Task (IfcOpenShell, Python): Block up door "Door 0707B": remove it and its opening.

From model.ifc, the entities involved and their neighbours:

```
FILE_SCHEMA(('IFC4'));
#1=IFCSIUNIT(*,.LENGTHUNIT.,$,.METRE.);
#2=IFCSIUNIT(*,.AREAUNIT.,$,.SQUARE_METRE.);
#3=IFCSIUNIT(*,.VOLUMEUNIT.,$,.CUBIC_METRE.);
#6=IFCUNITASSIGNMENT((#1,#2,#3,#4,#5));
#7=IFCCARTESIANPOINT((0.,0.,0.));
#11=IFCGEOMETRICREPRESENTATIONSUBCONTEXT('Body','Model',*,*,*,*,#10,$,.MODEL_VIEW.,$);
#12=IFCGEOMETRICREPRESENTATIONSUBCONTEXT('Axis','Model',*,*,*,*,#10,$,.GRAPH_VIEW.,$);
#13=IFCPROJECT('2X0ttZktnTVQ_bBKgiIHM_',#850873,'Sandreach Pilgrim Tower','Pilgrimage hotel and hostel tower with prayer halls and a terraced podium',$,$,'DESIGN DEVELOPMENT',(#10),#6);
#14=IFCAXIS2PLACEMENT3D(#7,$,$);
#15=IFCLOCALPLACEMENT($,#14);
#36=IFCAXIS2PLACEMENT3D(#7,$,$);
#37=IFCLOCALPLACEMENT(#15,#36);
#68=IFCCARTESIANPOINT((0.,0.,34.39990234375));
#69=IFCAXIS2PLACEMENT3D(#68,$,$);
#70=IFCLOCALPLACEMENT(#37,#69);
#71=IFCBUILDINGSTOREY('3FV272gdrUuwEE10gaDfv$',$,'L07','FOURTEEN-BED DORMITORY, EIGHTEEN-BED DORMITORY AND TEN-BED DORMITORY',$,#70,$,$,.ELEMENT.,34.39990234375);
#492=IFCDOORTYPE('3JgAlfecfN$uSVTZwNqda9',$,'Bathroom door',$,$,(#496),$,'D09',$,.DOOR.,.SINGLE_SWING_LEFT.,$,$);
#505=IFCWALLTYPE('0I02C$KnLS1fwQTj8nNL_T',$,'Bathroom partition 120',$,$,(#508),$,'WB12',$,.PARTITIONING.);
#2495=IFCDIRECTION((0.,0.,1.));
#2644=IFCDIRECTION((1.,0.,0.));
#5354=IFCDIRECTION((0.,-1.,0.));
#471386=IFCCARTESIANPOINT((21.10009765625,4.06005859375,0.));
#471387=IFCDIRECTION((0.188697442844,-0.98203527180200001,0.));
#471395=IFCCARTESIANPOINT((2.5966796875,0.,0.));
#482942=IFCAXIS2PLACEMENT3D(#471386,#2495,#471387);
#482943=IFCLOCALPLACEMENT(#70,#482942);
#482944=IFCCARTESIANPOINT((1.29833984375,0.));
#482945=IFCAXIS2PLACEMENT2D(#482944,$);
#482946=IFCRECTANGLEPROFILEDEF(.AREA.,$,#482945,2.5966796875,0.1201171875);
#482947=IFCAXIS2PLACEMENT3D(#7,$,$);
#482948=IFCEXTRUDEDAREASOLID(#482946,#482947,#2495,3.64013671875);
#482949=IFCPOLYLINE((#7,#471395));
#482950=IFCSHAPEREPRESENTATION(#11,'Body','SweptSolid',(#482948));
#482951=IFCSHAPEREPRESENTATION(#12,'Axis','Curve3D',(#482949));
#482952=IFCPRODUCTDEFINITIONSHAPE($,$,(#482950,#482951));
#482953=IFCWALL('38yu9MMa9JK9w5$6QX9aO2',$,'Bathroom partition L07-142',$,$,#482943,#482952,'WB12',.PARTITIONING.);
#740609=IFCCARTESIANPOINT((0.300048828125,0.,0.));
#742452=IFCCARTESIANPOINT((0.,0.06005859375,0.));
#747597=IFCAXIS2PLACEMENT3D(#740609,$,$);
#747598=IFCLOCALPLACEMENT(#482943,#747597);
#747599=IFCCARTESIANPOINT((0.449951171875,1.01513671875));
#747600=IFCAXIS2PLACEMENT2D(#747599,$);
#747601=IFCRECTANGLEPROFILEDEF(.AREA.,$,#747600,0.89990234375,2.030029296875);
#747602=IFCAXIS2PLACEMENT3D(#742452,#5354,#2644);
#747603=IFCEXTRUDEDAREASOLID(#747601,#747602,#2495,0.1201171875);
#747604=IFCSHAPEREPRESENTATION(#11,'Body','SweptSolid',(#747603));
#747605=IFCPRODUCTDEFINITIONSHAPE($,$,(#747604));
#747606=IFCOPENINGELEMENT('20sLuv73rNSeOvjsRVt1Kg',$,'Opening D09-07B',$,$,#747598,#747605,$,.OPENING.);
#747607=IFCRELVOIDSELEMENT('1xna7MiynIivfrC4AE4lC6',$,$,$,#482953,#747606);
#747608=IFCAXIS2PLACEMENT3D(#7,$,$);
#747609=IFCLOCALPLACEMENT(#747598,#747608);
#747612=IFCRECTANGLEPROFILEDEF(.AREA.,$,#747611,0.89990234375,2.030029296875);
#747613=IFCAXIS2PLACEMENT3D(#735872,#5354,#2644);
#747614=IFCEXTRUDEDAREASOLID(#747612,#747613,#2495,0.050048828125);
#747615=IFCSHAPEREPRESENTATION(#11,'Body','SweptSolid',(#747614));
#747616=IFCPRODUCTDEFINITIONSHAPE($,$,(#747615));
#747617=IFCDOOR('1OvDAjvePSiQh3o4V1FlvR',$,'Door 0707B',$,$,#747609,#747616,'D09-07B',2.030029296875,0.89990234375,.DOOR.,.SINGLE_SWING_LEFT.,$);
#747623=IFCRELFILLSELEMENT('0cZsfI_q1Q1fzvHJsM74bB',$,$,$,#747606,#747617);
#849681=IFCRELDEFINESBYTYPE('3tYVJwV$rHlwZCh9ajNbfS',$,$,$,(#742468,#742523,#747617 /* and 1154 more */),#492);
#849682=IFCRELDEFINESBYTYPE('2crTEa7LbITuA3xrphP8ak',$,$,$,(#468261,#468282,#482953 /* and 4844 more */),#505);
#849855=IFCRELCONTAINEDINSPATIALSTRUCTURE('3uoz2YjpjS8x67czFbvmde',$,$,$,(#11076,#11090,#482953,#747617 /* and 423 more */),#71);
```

```python
import ifcopenshell
import ifcopenshell.api.feature
import ifcopenshell.api.root
import ifcopenshell.geom
import ifcopenshell.util.shape

model = ifcopenshell.open("model.ifc")
settings = ifcopenshell.geom.settings()


def volume(element):
    """Net volume in cubic metres, openings subtracted."""
    shape = ifcopenshell.geom.create_shape(settings, element)
    return ifcopenshell.util.shape.get_volume(shape.geometry)


door = model.by_guid("1OvDAjvePSiQh3o4V1FlvR")
opening = door.FillsVoids[0].RelatingOpeningElement
wall = opening.VoidsElements[0].RelatingBuildingElement
before = volume(wall)

ifcopenshell.api.root.remove_product(model, product=door)
ifcopenshell.api.feature.remove_feature(model, feature=opening)

after = volume(wall)

print(f"wall volume {before:.3f} -> {after:.3f} m3")

model.write("model_rev.ifc")
```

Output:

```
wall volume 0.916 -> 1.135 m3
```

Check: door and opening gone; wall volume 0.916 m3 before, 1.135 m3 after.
